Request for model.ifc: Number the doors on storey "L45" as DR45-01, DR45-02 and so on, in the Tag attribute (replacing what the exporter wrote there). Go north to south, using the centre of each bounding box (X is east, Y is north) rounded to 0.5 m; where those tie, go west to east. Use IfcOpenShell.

First a look at what the model holds.

```python
import ifcopenshell
import ifcopenshell.util.element
import ifcopenshell.util.placement

model = ifcopenshell.open("model.ifc")
print(model.schema)
storey = next(s for s in model.by_type("IfcBuildingStorey") if s.Name == "L45")
doors = [e for e in ifcopenshell.util.element.get_decomposition(storey) if e.is_a("IfcDoor")]
for e in sorted(doors, key=lambda e: e.id()):
    origin = ifcopenshell.util.placement.get_local_placement(e.ObjectPlacement)[:3, 3]
    print(e.id(), e.Tag, e.Name, origin.round(2) + 0.0, sep=" | ")
```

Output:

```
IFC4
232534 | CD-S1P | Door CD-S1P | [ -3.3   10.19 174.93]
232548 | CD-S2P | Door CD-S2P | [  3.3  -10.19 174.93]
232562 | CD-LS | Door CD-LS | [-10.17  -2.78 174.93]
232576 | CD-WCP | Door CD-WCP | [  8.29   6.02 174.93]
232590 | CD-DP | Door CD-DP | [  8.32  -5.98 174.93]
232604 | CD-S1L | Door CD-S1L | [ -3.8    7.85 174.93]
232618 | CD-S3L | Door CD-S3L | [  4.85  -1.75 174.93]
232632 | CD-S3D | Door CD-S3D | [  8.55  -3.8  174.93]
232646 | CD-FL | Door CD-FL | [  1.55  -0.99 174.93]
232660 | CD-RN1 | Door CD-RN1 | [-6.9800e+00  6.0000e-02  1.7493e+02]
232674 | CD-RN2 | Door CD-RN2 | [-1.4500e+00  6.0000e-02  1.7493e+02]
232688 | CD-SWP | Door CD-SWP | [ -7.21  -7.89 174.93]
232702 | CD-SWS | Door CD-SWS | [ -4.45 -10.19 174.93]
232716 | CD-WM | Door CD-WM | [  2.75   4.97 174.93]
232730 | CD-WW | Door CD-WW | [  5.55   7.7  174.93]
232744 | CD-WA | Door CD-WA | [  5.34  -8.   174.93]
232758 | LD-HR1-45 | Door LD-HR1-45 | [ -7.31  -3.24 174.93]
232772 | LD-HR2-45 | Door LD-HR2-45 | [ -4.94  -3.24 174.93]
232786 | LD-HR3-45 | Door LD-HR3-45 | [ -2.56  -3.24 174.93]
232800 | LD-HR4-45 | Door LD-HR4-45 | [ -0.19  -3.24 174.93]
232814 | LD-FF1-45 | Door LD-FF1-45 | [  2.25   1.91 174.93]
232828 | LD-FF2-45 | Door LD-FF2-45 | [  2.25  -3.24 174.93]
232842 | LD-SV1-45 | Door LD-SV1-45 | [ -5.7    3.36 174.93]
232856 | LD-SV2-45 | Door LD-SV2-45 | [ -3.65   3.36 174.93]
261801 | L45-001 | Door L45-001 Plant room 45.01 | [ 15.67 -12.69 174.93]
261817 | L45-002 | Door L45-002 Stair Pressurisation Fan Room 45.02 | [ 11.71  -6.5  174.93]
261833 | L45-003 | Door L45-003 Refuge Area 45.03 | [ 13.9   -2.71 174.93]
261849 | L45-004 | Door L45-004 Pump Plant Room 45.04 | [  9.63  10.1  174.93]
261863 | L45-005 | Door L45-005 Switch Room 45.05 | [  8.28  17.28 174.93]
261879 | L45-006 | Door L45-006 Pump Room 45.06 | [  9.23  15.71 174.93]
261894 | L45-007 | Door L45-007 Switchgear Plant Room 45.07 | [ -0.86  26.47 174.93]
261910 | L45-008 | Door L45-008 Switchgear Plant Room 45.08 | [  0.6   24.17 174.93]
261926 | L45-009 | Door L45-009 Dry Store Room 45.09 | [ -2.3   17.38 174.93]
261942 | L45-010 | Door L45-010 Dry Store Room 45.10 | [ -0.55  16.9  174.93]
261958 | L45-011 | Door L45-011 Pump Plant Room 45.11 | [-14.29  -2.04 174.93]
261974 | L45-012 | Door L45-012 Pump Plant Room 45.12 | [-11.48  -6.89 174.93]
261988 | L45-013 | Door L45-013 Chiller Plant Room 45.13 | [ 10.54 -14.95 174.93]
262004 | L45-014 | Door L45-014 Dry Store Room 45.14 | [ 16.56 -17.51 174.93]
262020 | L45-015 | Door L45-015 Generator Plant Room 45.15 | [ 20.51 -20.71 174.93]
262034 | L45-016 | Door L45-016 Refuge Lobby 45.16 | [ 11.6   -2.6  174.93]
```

```python
import ifcopenshell
import ifcopenshell.geom
import ifcopenshell.util.element
import ifcopenshell.util.shape

model = ifcopenshell.open("model.ifc")
settings = ifcopenshell.geom.settings()
settings.set("use-world-coords", True)


def centre(element):
    shape = ifcopenshell.geom.create_shape(settings, element)
    return ifcopenshell.util.shape.get_bbox_centroid(shape.geometry)


storey = next(s for s in model.by_type("IfcBuildingStorey") if s.Name == "L45")
doors = [e for e in ifcopenshell.util.element.get_decomposition(storey) if e.is_a("IfcDoor")]

# Insertion points can sit at a corner or the storey origin, so sort by the geometry (in metres).
centres = {e: centre(e) for e in doors}
doors.sort(key=lambda e: (-round(centres[e][1] / 0.5), centres[e][0]))

for i, e in enumerate(doors, start=1):
    number = f"DR45-{i:02d}"
    e.Tag = number
    print(e.id(), number)

model.write("model_v2.ifc")
```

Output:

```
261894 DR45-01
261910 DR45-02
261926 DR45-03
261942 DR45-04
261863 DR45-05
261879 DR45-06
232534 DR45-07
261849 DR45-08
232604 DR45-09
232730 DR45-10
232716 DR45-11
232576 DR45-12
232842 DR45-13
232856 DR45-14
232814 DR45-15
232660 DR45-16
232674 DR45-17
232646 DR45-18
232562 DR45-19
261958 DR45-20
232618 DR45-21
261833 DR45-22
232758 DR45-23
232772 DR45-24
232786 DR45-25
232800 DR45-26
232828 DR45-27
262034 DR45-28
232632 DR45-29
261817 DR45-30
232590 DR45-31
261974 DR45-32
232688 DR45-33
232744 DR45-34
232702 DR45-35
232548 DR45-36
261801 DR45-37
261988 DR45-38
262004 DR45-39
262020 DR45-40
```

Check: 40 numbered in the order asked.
